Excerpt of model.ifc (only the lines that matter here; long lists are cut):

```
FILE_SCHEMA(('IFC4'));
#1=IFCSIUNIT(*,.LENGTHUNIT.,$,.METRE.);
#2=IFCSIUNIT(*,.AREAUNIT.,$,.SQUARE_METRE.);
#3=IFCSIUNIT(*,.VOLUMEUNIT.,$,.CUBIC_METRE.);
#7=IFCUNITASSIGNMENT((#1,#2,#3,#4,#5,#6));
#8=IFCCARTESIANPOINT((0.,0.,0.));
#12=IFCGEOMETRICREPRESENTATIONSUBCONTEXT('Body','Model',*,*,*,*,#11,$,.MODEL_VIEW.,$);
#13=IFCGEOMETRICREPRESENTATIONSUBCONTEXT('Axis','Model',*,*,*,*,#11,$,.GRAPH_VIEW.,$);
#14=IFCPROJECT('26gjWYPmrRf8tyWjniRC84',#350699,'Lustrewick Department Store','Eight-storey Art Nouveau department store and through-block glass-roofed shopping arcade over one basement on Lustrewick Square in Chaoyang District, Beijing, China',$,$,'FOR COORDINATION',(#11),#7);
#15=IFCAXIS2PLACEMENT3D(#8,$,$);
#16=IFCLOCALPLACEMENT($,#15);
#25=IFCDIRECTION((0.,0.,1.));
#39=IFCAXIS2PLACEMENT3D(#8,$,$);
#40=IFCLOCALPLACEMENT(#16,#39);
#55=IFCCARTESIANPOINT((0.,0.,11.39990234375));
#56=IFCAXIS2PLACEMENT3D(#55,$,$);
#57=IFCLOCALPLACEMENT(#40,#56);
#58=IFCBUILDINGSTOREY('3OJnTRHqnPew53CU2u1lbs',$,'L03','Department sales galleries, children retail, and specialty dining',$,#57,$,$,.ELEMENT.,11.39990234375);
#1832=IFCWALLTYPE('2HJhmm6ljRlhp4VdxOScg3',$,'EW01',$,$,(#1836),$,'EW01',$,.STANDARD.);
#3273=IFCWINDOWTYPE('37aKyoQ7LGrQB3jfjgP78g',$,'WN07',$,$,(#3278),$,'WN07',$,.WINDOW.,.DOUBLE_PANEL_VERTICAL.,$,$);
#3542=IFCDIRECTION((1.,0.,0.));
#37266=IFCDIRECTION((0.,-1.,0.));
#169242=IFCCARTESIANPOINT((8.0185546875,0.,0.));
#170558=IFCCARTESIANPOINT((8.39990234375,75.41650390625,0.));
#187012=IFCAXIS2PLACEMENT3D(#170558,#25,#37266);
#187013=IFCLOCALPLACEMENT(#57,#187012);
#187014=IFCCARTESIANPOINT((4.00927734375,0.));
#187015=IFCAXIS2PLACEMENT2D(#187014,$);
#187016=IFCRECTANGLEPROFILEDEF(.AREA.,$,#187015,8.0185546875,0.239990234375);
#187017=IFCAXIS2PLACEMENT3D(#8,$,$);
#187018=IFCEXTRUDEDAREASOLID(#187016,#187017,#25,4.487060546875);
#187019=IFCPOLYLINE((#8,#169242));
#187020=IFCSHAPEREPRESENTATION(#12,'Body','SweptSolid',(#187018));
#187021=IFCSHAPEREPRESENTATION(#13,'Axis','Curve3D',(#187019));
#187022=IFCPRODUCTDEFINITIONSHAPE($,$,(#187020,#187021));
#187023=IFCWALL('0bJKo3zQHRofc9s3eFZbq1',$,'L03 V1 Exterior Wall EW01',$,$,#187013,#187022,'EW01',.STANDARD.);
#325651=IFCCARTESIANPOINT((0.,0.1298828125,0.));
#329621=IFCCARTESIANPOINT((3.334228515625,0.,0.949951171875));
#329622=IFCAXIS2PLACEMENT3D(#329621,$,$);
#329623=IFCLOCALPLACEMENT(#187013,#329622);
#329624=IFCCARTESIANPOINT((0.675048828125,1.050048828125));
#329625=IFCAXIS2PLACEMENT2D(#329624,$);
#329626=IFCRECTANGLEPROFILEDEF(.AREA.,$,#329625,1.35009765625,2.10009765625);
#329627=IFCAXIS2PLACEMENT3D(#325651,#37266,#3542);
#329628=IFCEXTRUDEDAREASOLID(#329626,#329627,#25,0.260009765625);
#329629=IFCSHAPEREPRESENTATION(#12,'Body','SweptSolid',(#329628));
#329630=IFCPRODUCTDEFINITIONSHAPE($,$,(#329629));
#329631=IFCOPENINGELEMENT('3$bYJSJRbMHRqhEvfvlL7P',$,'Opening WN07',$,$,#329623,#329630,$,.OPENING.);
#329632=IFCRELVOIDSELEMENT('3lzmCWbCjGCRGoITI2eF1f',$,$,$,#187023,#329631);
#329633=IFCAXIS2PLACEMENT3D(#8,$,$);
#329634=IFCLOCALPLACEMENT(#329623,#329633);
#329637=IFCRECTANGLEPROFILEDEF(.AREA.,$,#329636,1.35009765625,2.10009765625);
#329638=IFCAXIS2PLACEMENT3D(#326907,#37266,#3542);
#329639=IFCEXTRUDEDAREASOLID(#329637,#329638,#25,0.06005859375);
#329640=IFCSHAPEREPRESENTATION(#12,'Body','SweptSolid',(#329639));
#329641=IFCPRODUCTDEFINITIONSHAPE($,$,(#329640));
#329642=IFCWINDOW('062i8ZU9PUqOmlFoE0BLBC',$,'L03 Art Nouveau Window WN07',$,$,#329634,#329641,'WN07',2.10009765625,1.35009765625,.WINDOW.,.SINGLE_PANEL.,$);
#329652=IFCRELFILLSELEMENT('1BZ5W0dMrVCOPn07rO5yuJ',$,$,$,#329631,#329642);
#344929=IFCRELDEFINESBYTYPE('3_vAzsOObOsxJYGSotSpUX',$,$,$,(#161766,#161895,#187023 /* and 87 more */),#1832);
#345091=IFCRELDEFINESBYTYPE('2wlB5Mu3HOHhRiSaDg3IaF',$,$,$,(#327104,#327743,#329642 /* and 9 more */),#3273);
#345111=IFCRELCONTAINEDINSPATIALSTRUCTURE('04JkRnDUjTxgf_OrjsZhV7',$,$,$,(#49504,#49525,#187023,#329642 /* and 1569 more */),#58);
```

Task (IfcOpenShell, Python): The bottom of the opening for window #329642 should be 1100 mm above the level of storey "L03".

```python
import numpy as np
import ifcopenshell
import ifcopenshell.api.geometry
import ifcopenshell.geom
import ifcopenshell.util.element
import ifcopenshell.util.placement
import ifcopenshell.util.shape
import ifcopenshell.util.unit

model = ifcopenshell.open("model.ifc")
unit_scale = ifcopenshell.util.unit.calculate_unit_scale(model)

window = model.by_guid("062i8ZU9PUqOmlFoE0BLBC")
opening = window.FillsVoids[0].RelatingOpeningElement
storey = ifcopenshell.util.element.get_container(window, ifc_class="IfcBuildingStorey")
level = ifcopenshell.util.placement.get_local_placement(storey.ObjectPlacement)[2, 3]

# The opening's origin need not be at the sill, so measure its lowest point.
shape = ifcopenshell.geom.create_shape(ifcopenshell.geom.settings(), opening)
bottom = ifcopenshell.util.shape.get_shape_bottom_elevation(shape, shape.geometry) / unit_scale
dz = level + 1.1 - bottom

shift = np.array([0.0, 0.0, dz])
# The window is placed relative to its opening, so it follows when the opening moves.
matrix = ifcopenshell.util.placement.get_local_placement(opening.ObjectPlacement)
matrix[:3, 3] += shift
ifcopenshell.api.geometry.edit_object_placement(
    model, product=opening, matrix=matrix, is_si=False, should_transform_children=True
)

print(f"moved by {dz * unit_scale:+.3f} m")

model.write("model-out.ifc")
```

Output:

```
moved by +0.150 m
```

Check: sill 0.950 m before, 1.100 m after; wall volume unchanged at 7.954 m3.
